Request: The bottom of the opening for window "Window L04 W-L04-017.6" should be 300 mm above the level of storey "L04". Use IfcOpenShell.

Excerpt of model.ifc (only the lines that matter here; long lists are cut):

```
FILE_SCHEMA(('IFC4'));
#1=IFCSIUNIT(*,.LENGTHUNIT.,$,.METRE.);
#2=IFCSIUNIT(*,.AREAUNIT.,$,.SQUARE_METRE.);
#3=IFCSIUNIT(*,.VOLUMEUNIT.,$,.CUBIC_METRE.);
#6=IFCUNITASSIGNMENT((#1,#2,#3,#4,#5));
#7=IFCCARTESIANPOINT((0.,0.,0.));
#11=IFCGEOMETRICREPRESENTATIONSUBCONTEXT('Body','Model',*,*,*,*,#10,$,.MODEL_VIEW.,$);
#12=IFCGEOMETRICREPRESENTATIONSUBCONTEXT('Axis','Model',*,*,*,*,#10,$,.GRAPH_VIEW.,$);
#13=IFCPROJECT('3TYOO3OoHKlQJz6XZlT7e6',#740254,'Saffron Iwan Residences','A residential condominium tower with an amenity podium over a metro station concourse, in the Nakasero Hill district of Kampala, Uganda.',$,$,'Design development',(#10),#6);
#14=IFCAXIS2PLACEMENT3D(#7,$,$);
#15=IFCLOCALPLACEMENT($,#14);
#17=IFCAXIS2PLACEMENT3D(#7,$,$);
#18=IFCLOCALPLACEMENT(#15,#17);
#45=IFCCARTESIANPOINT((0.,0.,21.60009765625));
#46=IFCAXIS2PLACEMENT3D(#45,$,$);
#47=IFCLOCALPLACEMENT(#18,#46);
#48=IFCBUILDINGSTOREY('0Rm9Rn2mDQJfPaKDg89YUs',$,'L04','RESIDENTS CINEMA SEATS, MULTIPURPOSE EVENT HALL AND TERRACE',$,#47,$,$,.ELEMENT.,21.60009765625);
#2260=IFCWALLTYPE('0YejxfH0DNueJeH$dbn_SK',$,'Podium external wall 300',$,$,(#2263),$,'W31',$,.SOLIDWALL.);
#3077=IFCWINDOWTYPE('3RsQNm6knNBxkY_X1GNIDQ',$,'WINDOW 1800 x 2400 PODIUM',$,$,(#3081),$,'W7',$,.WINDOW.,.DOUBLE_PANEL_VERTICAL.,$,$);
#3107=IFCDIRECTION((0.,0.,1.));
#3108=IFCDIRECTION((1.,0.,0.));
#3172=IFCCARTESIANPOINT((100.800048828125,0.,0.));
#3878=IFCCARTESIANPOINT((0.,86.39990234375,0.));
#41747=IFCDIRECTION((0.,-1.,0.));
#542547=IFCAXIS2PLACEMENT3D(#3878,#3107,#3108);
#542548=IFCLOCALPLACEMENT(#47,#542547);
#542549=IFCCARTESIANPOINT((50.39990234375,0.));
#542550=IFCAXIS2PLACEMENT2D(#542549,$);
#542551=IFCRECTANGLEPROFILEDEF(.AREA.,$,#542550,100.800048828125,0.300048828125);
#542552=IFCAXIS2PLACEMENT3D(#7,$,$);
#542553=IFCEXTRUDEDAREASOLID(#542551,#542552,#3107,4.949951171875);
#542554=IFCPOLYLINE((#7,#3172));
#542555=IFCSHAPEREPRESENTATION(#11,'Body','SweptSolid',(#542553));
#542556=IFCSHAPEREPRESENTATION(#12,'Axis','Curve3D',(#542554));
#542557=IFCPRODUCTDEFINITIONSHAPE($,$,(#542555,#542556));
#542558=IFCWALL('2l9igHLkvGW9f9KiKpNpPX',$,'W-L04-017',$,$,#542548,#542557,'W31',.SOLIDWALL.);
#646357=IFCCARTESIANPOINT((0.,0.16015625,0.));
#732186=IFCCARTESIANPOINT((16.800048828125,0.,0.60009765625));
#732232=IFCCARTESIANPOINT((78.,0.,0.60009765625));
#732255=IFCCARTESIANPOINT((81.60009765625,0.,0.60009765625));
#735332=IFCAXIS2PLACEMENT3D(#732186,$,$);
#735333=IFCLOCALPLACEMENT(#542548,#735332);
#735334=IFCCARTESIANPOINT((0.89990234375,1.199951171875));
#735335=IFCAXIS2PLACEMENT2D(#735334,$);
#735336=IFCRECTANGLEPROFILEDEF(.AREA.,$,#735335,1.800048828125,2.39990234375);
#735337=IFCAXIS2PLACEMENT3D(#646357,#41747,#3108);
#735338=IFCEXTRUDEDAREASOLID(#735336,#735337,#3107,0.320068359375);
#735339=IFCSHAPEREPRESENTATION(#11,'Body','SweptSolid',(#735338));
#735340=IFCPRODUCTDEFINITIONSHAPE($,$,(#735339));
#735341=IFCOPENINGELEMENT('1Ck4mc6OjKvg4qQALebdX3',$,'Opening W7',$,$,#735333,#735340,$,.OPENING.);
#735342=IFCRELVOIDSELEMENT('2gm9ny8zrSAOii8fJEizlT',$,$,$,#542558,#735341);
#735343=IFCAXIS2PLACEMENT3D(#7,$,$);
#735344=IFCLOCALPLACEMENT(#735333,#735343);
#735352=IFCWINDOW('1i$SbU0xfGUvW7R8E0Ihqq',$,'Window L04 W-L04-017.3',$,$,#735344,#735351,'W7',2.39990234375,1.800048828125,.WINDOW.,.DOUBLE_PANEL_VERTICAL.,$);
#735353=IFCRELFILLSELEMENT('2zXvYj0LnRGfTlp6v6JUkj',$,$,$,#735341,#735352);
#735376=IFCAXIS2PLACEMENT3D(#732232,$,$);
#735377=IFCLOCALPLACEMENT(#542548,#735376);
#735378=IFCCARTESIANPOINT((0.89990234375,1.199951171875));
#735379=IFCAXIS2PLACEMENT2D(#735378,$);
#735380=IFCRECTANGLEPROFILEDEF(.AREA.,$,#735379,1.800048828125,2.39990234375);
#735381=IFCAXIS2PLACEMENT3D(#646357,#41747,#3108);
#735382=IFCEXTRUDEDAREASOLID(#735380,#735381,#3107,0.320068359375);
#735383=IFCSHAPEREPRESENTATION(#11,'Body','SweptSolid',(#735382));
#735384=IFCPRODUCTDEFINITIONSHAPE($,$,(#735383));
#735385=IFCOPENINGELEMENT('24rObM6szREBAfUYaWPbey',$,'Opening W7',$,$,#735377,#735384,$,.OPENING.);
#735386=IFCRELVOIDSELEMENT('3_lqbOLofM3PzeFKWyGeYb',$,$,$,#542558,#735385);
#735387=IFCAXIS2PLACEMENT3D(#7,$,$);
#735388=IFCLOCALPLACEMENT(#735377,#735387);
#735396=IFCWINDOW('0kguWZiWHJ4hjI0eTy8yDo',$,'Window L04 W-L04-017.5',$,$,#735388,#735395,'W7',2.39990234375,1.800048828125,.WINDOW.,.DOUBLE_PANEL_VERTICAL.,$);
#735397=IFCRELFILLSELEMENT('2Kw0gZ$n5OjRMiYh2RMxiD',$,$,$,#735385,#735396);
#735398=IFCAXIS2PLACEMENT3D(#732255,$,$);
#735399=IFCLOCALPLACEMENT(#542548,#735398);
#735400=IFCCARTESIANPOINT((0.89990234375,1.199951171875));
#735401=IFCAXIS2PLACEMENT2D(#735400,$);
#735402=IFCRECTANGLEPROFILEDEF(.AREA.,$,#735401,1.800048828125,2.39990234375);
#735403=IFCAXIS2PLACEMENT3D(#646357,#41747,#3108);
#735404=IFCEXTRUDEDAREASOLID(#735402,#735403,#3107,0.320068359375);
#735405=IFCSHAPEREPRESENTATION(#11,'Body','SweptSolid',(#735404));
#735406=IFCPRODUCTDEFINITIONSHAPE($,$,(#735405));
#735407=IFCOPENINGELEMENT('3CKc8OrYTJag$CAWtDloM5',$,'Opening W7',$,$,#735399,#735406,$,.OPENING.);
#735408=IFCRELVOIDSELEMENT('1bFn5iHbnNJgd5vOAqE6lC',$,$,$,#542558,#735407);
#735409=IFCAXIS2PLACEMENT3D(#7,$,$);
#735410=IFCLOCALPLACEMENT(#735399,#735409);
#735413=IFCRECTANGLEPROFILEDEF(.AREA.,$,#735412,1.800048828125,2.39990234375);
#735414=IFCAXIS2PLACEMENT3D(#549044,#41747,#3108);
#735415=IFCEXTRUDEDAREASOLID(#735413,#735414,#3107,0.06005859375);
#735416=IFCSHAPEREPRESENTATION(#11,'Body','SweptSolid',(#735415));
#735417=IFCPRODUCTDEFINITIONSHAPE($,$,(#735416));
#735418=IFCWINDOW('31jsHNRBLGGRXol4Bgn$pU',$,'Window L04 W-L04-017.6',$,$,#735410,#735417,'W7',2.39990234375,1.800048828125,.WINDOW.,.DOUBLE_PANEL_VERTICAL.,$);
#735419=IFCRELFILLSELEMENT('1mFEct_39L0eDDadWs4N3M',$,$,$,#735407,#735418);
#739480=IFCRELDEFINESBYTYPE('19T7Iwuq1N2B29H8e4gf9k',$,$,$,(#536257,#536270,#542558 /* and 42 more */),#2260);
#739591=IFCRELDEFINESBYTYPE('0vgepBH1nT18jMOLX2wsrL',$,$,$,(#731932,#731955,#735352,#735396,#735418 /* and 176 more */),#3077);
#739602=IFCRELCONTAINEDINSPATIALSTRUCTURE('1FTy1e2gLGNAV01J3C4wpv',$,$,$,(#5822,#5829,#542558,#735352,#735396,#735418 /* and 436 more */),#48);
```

```python
import numpy as np
import ifcopenshell
import ifcopenshell.api.geometry
import ifcopenshell.geom
import ifcopenshell.util.element
import ifcopenshell.util.placement
import ifcopenshell.util.shape
import ifcopenshell.util.unit

model = ifcopenshell.open("model.ifc")
unit_scale = ifcopenshell.util.unit.calculate_unit_scale(model)

window = model.by_guid("31jsHNRBLGGRXol4Bgn$pU")
opening = window.FillsVoids[0].RelatingOpeningElement
storey = ifcopenshell.util.element.get_container(window, ifc_class="IfcBuildingStorey")
level = ifcopenshell.util.placement.get_local_placement(storey.ObjectPlacement)[2, 3]

# The opening's origin need not be at the sill, so measure its lowest point.
shape = ifcopenshell.geom.create_shape(ifcopenshell.geom.settings(), opening)
bottom = ifcopenshell.util.shape.get_shape_bottom_elevation(shape, shape.geometry) / unit_scale
dz = level + 0.3 / unit_scale - bottom

shift = np.array([0.0, 0.0, dz])
# The window is placed relative to its opening, so it follows when the opening moves.
matrix = ifcopenshell.util.placement.get_local_placement(opening.ObjectPlacement)
matrix[:3, 3] += shift
ifcopenshell.api.geometry.edit_object_placement(
    model, product=opening, matrix=matrix, is_si=False, should_transform_children=True
)

print(f"moved by {dz * unit_scale:+.3f} m")

model.write("model_rev.ifc")
```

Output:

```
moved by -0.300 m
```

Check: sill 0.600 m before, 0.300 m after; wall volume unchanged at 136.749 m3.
